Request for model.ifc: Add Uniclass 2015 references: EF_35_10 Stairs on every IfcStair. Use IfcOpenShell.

First a look at what the model holds.

```python
import ifcopenshell

model = ifcopenshell.open("model.ifc")
print(model.schema)
print("classifications:", [c.Name for c in model.by_type("IfcClassification")])
for ifc_class in ("IfcDoor", "IfcRoof", "IfcStair", "IfcWall", "IfcWindow"):
    print(ifc_class, len(model.by_type(ifc_class)))
```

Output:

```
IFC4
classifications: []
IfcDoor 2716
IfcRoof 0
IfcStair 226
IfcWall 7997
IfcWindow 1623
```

```python
import ifcopenshell
import ifcopenshell.api.classification

model = ifcopenshell.open("model.ifc")

system = ifcopenshell.api.classification.add_classification(model, classification="Uniclass 2015")

codes = {
    "IfcStair": ("EF_35_10", "Stairs"),
}
for ifc_class, (code, name) in codes.items():
    products = model.by_type(ifc_class)
    ifcopenshell.api.classification.add_reference(
        model, products=products, classification=system, identification=code, name=name
    )
    print(code, len(products))

model.write("model_edited.ifc")
```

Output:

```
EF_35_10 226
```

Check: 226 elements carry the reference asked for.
